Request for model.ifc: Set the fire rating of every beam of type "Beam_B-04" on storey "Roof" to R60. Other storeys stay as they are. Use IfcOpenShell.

First a look at what the model holds.

```python
import ifcopenshell
import ifcopenshell.util.element

model = ifcopenshell.open("model.ifc")
print(model.schema)
storey = next(s for s in model.by_type("IfcBuildingStorey") if s.Name == "Roof")
beams = [e for e in ifcopenshell.util.element.get_decomposition(storey) if e.is_a("IfcBeam")]
seen = {}
for e in beams:
    element_type = ifcopenshell.util.element.get_type(e)
    key = (element_type.Name if element_type != e and element_type else None, ifcopenshell.util.element.get_pset(e, "Pset_BeamCommon", "FireRating"))
    seen[key] = seen.get(key, 0) + 1
for (name, value), count in sorted(seen.items(), key=str):
    print(count, "x", name, "|", value)
```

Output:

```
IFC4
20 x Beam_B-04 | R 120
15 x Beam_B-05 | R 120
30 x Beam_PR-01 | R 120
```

```python
import ifcopenshell
import ifcopenshell.api.pset
import ifcopenshell.util.element

model = ifcopenshell.open("model.ifc")

storey = next(s for s in model.by_type("IfcBuildingStorey") if s.Name == "Roof")
beams = [e for e in ifcopenshell.util.element.get_decomposition(storey) if e.is_a("IfcBeam")]

count = 0
for e in beams:
    element_type = ifcopenshell.util.element.get_type(e)
    if element_type in (None, e) or element_type.Name != "Beam_B-04":
        continue
    # add_pset returns the element's existing set when there is one.
    pset = ifcopenshell.api.pset.add_pset(model, product=e, name="Pset_BeamCommon")
    ifcopenshell.api.pset.edit_pset(model, pset=pset, properties={"FireRating": "R60"})
    count += 1

print(count, "beams updated")

model.write("model_v2.ifc")
```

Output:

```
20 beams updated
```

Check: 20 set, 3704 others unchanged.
